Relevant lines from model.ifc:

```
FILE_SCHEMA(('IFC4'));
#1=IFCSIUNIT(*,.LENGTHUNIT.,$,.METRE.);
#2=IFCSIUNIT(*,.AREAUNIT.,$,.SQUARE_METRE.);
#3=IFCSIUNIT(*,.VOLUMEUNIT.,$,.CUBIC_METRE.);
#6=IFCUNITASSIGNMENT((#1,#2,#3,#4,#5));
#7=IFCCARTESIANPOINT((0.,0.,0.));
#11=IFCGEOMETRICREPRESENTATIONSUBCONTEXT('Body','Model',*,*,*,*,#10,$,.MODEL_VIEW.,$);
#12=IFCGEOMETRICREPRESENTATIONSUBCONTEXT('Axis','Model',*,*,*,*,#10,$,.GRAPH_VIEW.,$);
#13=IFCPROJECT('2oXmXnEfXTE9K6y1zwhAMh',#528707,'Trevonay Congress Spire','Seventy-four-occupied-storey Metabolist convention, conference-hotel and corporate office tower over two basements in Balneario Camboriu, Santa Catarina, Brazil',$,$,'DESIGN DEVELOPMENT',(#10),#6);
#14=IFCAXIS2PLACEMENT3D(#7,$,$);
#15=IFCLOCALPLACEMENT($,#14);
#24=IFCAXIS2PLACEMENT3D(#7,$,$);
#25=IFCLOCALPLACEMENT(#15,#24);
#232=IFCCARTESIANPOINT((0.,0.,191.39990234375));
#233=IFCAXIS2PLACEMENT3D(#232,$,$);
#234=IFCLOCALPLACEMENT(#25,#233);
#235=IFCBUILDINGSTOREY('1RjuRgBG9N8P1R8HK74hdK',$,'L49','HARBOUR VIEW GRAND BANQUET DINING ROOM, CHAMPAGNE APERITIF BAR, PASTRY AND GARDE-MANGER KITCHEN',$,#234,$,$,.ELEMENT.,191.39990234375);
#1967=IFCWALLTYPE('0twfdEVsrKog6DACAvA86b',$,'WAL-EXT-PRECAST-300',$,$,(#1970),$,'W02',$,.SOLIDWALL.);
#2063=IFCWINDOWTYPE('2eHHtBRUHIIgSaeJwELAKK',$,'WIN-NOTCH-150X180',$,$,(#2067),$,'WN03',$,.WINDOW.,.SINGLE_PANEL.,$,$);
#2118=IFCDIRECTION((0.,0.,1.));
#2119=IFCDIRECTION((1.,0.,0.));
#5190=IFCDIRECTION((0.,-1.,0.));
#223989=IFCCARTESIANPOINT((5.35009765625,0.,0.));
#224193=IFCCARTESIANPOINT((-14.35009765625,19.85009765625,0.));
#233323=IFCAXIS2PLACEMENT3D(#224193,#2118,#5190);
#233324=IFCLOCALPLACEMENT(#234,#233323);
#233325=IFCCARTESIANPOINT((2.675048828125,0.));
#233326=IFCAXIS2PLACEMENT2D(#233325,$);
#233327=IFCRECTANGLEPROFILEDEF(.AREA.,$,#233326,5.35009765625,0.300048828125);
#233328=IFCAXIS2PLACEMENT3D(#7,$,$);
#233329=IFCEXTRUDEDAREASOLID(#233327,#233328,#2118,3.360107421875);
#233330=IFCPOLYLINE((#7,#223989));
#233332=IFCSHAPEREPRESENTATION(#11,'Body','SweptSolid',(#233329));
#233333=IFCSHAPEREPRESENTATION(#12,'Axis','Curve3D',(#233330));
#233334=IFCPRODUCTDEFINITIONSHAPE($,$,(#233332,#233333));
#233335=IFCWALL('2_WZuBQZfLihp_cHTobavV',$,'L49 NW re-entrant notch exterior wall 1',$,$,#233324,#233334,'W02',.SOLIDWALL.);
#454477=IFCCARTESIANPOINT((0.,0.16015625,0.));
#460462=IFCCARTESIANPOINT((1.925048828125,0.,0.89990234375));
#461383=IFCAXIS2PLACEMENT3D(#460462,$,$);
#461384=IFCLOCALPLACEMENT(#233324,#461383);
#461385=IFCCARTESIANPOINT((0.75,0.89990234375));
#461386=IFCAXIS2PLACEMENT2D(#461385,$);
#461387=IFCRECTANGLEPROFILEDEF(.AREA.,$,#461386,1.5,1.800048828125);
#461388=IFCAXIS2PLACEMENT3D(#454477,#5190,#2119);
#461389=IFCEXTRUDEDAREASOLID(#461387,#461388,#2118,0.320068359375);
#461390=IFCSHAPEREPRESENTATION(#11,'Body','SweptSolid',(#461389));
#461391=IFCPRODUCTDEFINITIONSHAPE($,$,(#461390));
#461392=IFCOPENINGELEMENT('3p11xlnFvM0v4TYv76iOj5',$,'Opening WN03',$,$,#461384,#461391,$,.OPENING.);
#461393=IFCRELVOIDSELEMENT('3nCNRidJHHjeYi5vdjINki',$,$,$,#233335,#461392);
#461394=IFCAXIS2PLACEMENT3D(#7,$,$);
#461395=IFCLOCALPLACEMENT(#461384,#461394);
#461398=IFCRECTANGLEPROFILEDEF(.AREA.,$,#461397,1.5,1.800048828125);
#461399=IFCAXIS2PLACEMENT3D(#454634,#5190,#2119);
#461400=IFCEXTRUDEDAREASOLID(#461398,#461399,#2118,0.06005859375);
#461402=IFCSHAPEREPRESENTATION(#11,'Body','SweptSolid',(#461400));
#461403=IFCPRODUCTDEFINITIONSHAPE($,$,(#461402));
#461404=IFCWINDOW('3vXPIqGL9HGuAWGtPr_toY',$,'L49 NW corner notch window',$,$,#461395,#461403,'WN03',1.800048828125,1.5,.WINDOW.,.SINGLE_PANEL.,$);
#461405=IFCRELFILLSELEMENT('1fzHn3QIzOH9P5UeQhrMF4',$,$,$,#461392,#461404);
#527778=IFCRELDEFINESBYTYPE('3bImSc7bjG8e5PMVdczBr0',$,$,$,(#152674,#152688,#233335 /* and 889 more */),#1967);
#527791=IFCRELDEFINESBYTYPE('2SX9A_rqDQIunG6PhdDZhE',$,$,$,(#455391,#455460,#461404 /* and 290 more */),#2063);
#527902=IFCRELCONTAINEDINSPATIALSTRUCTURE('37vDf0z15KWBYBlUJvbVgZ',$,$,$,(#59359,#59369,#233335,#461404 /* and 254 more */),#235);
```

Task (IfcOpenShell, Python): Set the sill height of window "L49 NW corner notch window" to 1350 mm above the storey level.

```python
import numpy as np
import ifcopenshell
import ifcopenshell.api.geometry
import ifcopenshell.geom
import ifcopenshell.util.element
import ifcopenshell.util.placement
import ifcopenshell.util.shape
import ifcopenshell.util.unit

model = ifcopenshell.open("model.ifc")
unit_scale = ifcopenshell.util.unit.calculate_unit_scale(model)

window = model.by_id(461404)
opening = window.FillsVoids[0].RelatingOpeningElement
storey = ifcopenshell.util.element.get_container(window, ifc_class="IfcBuildingStorey")
level = ifcopenshell.util.placement.get_local_placement(storey.ObjectPlacement)[2, 3]

# The opening's origin need not be at the sill, so measure its lowest point.
shape = ifcopenshell.geom.create_shape(ifcopenshell.geom.settings(), opening)
bottom = ifcopenshell.util.shape.get_shape_bottom_elevation(shape, shape.geometry) / unit_scale
dz = level + 1.35 - bottom

shift = np.array([0.0, 0.0, dz])
# The window is placed relative to its opening, so it follows when the opening moves.
matrix = ifcopenshell.util.placement.get_local_placement(opening.ObjectPlacement)
matrix[:3, 3] += shift
ifcopenshell.api.geometry.edit_object_placement(
    model, product=opening, matrix=matrix, is_si=False, should_transform_children=True
)

print(f"moved by {dz * unit_scale:+.3f} m")

model.write("model-out.ifc")
```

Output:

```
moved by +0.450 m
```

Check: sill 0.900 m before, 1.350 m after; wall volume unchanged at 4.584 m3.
